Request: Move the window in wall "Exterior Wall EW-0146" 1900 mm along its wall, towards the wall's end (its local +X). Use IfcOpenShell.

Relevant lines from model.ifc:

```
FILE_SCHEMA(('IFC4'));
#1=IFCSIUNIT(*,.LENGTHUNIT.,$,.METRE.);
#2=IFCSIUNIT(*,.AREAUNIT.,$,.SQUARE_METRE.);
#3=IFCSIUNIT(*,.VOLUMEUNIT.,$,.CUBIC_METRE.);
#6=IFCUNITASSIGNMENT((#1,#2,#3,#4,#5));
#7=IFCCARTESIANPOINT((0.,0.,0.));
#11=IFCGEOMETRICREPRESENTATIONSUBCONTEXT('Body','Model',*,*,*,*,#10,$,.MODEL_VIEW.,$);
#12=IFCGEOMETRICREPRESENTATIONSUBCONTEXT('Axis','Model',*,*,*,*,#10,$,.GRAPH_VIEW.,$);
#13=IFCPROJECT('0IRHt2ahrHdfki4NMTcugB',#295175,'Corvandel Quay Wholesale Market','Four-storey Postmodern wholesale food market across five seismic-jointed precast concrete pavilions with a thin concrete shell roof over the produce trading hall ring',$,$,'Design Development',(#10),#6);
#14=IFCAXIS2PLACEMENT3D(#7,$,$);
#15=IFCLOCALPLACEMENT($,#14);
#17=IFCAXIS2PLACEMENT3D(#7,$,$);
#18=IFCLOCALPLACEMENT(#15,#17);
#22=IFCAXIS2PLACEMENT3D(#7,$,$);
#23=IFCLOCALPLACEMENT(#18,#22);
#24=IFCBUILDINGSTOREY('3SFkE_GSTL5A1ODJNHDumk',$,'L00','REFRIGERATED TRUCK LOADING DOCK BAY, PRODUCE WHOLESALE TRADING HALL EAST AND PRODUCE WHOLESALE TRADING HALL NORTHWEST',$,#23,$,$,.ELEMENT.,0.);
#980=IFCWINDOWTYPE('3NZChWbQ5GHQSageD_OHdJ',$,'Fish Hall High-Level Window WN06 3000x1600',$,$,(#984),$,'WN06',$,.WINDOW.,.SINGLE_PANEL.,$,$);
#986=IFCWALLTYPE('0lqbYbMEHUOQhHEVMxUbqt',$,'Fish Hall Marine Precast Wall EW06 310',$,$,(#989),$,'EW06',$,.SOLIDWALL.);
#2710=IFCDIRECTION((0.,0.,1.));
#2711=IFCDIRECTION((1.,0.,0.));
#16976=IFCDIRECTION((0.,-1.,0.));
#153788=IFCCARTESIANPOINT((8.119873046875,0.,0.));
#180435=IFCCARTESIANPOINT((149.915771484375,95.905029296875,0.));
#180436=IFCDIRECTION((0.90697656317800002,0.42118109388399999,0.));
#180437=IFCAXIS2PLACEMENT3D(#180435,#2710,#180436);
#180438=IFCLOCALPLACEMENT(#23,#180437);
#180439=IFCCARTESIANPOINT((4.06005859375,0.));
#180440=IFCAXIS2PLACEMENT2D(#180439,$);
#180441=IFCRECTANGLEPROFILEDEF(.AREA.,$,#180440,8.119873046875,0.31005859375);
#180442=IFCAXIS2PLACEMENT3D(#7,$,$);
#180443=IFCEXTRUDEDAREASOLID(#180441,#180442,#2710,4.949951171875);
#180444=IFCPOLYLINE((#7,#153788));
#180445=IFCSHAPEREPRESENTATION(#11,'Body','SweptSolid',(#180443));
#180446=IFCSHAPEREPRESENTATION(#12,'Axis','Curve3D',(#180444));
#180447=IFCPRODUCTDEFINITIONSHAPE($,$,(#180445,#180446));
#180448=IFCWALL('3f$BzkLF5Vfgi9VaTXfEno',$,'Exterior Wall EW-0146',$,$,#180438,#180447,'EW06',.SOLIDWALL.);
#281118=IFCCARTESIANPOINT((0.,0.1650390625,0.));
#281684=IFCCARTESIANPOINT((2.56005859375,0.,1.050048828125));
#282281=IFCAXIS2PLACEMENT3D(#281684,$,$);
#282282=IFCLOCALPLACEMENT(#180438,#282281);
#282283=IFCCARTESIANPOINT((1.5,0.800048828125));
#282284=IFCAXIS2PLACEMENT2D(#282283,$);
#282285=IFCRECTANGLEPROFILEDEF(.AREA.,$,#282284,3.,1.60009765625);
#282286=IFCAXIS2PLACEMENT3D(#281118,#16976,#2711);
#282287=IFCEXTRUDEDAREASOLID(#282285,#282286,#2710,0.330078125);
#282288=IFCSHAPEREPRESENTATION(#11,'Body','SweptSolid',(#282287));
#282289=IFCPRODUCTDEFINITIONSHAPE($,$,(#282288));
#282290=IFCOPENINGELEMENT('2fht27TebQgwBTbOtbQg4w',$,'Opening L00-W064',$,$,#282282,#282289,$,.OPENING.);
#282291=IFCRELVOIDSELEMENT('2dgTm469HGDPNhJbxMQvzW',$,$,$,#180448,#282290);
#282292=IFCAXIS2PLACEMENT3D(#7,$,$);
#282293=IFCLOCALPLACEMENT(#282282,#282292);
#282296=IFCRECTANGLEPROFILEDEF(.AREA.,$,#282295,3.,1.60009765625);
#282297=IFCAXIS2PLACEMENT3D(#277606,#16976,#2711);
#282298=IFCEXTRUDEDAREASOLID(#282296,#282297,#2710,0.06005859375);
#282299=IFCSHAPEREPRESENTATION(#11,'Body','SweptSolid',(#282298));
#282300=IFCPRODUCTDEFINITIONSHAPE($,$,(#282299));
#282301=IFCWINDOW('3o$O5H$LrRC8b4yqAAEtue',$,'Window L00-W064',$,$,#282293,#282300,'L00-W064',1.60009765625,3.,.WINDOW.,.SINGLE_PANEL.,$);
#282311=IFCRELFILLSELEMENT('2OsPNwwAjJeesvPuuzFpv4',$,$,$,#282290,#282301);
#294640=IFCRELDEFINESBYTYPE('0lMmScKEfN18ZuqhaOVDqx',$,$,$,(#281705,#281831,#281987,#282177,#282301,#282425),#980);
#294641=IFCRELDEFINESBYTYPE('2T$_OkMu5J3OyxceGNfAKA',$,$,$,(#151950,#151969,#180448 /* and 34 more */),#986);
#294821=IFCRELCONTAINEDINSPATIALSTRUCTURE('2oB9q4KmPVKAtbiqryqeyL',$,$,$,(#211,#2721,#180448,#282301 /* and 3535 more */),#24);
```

```python
import ifcopenshell
import ifcopenshell.api.geometry
import ifcopenshell.util.placement

model = ifcopenshell.open("model.ifc")

window = model.by_guid("3o$O5H$LrRC8b4yqAAEtue")
opening = window.FillsVoids[0].RelatingOpeningElement
wall = opening.VoidsElements[0].RelatingBuildingElement

wall_matrix = ifcopenshell.util.placement.get_local_placement(wall.ObjectPlacement)
shift = wall_matrix[:3, 0] * 1.9
before = ifcopenshell.util.placement.get_local_placement(window.ObjectPlacement)[:3, 3].copy()

# The window is placed relative to its opening, so it follows when the opening moves.
matrix = ifcopenshell.util.placement.get_local_placement(opening.ObjectPlacement)
matrix[:3, 3] += shift
ifcopenshell.api.geometry.edit_object_placement(
    model, product=opening, matrix=matrix, is_si=False, should_transform_children=True
)

after = ifcopenshell.util.placement.get_local_placement(window.ObjectPlacement)[:3, 3]
print("window moved by", (after - before).round(3) + 0.0)

model.write("model-out.ifc")
```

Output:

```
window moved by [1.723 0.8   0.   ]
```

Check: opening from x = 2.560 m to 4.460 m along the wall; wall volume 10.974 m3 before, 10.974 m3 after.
